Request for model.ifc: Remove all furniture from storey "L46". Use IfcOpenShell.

First a look at what the model holds.

```python
import ifcopenshell
import ifcopenshell.util.element

model = ifcopenshell.open("model.ifc")
print(model.schema)
storey = next(s for s in model.by_type("IfcBuildingStorey") if s.Name == "L46")
furniture = [e for e in ifcopenshell.util.element.get_decomposition(storey) if e.is_a("IfcFurnishingElement")]
seen = {}
for e in furniture:
    element_type = ifcopenshell.util.element.get_type(e)
    name = element_type.Name if element_type not in (None, e) else None
    seen[name] = seen.get(name, 0) + 1
for name, count in sorted(seen.items(), key=str):
    print(count, "x", name)
```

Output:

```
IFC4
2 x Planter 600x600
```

```python
import ifcopenshell
import ifcopenshell.api.root
import ifcopenshell.util.element

model = ifcopenshell.open("model.ifc")

storey = next(s for s in model.by_type("IfcBuildingStorey") if s.Name == "L46")
furniture = [e for e in ifcopenshell.util.element.get_decomposition(storey) if e.is_a("IfcFurnishingElement")]

for e in furniture:
    ifcopenshell.api.root.remove_product(model, product=e)
print(len(furniture), "removed")

model.write("model_v2.ifc")
```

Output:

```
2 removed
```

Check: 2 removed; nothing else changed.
